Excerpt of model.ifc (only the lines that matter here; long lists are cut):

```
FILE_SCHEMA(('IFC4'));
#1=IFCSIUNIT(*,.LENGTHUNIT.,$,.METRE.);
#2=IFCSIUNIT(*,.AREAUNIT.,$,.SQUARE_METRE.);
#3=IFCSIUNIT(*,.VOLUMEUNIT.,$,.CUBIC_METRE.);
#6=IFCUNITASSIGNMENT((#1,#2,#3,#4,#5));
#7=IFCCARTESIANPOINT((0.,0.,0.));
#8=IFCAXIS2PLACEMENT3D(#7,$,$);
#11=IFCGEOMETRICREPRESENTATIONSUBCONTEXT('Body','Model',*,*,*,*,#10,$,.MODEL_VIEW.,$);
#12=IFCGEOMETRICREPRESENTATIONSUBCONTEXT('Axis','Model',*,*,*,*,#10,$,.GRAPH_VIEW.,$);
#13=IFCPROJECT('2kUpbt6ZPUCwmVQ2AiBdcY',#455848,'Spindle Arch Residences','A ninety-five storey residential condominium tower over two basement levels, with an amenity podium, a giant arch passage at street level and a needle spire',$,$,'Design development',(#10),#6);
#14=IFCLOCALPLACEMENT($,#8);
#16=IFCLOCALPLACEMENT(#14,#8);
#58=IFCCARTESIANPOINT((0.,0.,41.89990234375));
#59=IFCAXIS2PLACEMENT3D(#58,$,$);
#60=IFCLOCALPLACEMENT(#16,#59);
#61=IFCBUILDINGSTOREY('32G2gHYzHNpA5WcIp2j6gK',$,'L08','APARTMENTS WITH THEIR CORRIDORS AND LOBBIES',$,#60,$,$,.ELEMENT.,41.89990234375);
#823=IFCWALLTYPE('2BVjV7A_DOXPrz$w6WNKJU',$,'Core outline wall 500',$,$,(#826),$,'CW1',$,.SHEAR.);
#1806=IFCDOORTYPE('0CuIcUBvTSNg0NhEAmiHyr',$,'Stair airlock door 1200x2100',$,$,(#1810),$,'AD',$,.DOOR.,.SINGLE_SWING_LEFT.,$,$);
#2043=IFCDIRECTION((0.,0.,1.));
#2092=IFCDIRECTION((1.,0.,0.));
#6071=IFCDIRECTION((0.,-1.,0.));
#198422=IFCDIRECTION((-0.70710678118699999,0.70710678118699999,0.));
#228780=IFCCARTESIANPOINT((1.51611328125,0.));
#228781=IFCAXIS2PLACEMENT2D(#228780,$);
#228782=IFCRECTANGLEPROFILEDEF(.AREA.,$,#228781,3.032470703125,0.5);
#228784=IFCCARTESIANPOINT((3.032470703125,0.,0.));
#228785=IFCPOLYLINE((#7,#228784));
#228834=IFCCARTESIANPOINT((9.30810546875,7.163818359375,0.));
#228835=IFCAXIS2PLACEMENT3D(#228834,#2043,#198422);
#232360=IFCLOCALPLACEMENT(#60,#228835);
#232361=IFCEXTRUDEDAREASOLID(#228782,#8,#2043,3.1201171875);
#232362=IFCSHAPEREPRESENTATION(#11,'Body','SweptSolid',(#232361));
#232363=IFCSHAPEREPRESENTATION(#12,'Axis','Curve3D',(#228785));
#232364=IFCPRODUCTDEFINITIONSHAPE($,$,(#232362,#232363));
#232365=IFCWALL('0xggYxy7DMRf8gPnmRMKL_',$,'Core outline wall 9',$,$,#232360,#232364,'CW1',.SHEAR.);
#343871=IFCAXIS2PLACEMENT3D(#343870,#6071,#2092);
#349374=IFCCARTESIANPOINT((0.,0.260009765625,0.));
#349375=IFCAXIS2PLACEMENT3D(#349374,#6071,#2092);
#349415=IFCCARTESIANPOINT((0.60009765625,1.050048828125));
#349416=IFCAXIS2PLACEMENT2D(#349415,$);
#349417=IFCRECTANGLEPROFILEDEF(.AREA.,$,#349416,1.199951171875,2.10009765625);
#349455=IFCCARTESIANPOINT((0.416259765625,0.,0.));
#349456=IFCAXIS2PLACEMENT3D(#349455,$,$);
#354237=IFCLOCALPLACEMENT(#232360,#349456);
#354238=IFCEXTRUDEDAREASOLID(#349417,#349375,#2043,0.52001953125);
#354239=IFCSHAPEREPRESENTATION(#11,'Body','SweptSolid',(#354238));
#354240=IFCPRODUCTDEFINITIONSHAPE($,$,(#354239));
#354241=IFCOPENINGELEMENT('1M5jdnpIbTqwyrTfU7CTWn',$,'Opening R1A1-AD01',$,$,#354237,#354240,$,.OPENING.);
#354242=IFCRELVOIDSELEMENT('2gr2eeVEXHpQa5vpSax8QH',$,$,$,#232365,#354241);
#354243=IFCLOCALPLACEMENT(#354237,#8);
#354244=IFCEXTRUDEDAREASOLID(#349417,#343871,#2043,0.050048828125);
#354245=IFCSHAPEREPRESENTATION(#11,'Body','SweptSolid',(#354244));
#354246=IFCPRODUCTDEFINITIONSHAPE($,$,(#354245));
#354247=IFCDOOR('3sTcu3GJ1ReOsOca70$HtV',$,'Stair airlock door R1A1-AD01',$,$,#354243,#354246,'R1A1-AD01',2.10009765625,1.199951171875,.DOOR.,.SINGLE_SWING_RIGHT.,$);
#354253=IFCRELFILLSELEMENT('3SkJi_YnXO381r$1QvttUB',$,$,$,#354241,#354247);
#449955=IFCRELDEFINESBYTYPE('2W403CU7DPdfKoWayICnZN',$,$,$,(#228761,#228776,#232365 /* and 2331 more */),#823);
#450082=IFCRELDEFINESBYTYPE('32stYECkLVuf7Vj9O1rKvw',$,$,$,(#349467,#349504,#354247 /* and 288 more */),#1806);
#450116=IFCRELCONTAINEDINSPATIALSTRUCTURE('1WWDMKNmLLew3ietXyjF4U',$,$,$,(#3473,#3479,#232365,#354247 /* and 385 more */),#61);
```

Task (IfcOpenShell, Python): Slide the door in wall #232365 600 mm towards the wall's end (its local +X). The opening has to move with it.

```python
import ifcopenshell
import ifcopenshell.api.geometry
import ifcopenshell.util.placement
import ifcopenshell.util.unit

model = ifcopenshell.open("model.ifc")
unit_scale = ifcopenshell.util.unit.calculate_unit_scale(model)

door = model.by_guid("3sTcu3GJ1ReOsOca70$HtV")
opening = door.FillsVoids[0].RelatingOpeningElement
wall = opening.VoidsElements[0].RelatingBuildingElement

wall_matrix = ifcopenshell.util.placement.get_local_placement(wall.ObjectPlacement)
shift = wall_matrix[:3, 0] * 0.6 / unit_scale
before = ifcopenshell.util.placement.get_local_placement(door.ObjectPlacement)[:3, 3].copy()

# The door is placed relative to its opening, so it follows when the opening moves.
matrix = ifcopenshell.util.placement.get_local_placement(opening.ObjectPlacement)
matrix[:3, 3] += shift
ifcopenshell.api.geometry.edit_object_placement(
    model, product=opening, matrix=matrix, is_si=False, should_transform_children=True
)

after = ifcopenshell.util.placement.get_local_placement(door.ObjectPlacement)[:3, 3]
print("door moved by", (after - before).round(3) + 0.0)

model.write("model_v2.ifc")
```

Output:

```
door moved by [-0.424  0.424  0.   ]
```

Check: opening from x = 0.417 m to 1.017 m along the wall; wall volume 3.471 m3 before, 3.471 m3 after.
